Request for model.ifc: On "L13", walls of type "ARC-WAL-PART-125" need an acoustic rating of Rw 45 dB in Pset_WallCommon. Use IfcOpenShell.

First a look at what the model holds.

```python
import ifcopenshell
import ifcopenshell.util.element

model = ifcopenshell.open("model.ifc")
print(model.schema)
storey = next(s for s in model.by_type("IfcBuildingStorey") if s.Name == "L13")
walls = [e for e in ifcopenshell.util.element.get_decomposition(storey) if e.is_a("IfcWall")]
seen = {}
for e in walls:
    element_type = ifcopenshell.util.element.get_type(e)
    key = (element_type.Name if element_type != e and element_type else None, ifcopenshell.util.element.get_pset(e, "Pset_WallCommon", "AcousticRating"))
    seen[key] = seen.get(key, 0) + 1
for (name, value), count in sorted(seen.items(), key=str):
    print(count, "x", name, "|", value)
```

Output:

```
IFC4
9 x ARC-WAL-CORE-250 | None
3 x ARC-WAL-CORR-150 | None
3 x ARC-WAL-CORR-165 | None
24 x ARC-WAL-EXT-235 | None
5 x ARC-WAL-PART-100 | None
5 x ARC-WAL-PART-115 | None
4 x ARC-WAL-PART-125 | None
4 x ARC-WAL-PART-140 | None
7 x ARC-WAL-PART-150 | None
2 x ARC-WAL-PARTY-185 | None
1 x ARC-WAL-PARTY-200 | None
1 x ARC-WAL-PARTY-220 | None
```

```python
import ifcopenshell
import ifcopenshell.api.pset
import ifcopenshell.util.element

model = ifcopenshell.open("model.ifc")

storey = next(s for s in model.by_type("IfcBuildingStorey") if s.Name == "L13")
walls = [e for e in ifcopenshell.util.element.get_decomposition(storey) if e.is_a("IfcWall")]

count = 0
for e in walls:
    element_type = ifcopenshell.util.element.get_type(e)
    if element_type in (None, e) or element_type.Name != "ARC-WAL-PART-125":
        continue
    # add_pset returns the element's existing set when there is one.
    pset = ifcopenshell.api.pset.add_pset(model, product=e, name="Pset_WallCommon")
    ifcopenshell.api.pset.edit_pset(model, pset=pset, properties={"AcousticRating": "Rw 45 dB"})
    count += 1

print(count, "walls updated")

model.write("model_rev.ifc")
```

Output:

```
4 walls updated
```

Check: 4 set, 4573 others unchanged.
